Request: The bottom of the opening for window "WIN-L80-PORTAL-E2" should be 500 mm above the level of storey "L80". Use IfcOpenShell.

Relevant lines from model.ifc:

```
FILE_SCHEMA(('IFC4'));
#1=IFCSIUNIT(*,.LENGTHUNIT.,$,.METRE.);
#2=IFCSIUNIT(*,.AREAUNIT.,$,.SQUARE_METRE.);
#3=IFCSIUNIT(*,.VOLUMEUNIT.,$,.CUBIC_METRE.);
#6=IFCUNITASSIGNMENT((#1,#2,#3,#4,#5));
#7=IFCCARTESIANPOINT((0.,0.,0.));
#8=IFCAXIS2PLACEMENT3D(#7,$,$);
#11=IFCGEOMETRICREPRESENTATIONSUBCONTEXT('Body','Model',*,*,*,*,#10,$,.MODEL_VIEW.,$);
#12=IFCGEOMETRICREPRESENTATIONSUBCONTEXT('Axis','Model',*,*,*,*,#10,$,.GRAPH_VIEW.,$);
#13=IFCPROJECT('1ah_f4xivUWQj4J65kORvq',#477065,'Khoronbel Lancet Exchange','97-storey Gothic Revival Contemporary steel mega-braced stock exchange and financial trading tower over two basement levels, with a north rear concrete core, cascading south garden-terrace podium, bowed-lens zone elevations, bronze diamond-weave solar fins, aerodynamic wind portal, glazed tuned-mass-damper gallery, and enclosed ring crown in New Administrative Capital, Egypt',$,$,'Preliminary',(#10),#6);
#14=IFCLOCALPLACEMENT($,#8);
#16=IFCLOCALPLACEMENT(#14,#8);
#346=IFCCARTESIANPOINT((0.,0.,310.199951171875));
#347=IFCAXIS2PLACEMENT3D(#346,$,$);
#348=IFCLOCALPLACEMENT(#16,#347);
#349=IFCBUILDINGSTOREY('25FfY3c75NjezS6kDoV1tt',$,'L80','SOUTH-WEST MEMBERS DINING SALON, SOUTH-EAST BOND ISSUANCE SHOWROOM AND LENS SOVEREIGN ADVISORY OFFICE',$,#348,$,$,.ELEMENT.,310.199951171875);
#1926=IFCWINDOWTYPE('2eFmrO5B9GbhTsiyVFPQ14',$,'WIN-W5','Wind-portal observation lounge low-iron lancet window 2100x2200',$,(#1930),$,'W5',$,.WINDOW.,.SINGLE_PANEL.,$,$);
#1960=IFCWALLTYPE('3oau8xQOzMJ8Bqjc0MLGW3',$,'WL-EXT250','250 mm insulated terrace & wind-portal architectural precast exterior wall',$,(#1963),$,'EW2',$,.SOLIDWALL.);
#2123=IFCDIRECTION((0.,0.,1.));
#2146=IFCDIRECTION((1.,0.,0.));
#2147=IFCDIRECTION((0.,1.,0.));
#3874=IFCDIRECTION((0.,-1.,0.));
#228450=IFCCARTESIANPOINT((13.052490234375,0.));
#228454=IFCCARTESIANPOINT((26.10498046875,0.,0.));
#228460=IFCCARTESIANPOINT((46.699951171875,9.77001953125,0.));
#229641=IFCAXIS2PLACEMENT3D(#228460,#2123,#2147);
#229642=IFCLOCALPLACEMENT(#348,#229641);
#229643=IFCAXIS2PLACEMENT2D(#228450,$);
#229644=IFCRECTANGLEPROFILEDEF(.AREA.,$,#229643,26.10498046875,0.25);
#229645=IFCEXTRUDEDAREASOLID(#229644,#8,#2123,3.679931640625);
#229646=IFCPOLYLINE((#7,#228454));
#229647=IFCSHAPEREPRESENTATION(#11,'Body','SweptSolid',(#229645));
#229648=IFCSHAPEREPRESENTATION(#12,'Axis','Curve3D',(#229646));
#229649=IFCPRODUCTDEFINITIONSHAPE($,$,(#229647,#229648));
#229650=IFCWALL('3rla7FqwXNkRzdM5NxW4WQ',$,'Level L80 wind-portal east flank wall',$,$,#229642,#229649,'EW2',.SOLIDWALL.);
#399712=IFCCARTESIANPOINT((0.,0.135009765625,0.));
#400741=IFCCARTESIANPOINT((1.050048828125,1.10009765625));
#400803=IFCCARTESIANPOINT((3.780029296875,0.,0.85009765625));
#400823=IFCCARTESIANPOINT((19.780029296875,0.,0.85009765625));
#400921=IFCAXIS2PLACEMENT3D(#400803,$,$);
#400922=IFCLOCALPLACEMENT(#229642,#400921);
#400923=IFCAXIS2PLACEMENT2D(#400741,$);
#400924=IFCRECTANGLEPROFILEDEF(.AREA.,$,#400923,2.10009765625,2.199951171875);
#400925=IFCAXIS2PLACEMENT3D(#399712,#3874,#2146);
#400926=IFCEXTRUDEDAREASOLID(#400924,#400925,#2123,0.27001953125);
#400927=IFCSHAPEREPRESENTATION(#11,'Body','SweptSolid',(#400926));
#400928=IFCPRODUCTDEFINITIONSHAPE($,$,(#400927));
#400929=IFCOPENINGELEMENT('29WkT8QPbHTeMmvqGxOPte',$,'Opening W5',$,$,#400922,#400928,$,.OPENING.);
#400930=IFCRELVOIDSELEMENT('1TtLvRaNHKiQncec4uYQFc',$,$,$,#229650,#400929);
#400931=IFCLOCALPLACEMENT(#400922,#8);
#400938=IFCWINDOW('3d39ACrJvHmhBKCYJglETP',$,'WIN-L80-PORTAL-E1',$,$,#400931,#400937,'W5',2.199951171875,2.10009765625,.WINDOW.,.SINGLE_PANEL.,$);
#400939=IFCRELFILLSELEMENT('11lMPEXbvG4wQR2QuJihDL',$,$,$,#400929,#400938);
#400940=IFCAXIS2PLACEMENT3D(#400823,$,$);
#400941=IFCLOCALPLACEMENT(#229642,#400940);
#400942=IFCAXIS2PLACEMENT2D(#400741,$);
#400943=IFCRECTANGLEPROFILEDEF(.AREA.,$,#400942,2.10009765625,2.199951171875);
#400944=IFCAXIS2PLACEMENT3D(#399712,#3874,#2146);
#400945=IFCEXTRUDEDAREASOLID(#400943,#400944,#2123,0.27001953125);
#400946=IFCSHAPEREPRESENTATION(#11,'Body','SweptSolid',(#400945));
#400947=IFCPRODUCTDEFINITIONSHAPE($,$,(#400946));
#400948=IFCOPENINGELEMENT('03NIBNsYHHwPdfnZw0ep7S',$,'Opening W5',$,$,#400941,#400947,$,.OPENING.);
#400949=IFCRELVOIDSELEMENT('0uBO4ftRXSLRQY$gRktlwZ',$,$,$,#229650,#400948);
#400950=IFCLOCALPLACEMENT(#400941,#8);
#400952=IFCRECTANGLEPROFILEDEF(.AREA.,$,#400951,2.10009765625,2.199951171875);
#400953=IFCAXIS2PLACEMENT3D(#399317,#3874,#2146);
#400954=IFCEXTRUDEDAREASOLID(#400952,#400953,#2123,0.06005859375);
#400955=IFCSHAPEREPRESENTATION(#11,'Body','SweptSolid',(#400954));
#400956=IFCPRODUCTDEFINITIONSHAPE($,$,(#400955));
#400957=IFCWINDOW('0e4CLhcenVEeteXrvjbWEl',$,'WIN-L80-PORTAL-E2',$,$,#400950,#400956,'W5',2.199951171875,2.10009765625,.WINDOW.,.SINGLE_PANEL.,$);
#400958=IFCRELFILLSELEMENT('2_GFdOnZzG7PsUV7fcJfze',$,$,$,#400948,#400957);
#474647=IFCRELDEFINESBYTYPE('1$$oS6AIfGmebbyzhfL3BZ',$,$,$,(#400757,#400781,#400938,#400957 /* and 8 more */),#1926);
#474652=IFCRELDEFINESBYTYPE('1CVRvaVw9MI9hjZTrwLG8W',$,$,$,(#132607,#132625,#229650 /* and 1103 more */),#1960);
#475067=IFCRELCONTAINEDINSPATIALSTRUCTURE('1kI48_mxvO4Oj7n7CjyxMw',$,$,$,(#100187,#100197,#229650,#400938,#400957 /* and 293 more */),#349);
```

```python
import numpy as np
import ifcopenshell
import ifcopenshell.api.geometry
import ifcopenshell.geom
import ifcopenshell.util.element
import ifcopenshell.util.placement
import ifcopenshell.util.shape
import ifcopenshell.util.unit

model = ifcopenshell.open("model.ifc")
unit_scale = ifcopenshell.util.unit.calculate_unit_scale(model)

window = model.by_id(400957)
opening = window.FillsVoids[0].RelatingOpeningElement
storey = ifcopenshell.util.element.get_container(window, ifc_class="IfcBuildingStorey")
level = ifcopenshell.util.placement.get_local_placement(storey.ObjectPlacement)[2, 3]

# The opening's origin need not be at the sill, so measure its lowest point.
shape = ifcopenshell.geom.create_shape(ifcopenshell.geom.settings(), opening)
bottom = ifcopenshell.util.shape.get_shape_bottom_elevation(shape, shape.geometry) / unit_scale
dz = level + 0.5 / unit_scale - bottom

shift = np.array([0.0, 0.0, dz])
# The window is placed relative to its opening, so it follows when the opening moves.
matrix = ifcopenshell.util.placement.get_local_placement(opening.ObjectPlacement)
matrix[:3, 3] += shift
ifcopenshell.api.geometry.edit_object_placement(
    model, product=opening, matrix=matrix, is_si=False, should_transform_children=True
)

print(f"moved by {dz * unit_scale:+.3f} m")

model.write("model_edited.ifc")
```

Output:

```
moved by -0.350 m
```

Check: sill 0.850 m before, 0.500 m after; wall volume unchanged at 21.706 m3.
